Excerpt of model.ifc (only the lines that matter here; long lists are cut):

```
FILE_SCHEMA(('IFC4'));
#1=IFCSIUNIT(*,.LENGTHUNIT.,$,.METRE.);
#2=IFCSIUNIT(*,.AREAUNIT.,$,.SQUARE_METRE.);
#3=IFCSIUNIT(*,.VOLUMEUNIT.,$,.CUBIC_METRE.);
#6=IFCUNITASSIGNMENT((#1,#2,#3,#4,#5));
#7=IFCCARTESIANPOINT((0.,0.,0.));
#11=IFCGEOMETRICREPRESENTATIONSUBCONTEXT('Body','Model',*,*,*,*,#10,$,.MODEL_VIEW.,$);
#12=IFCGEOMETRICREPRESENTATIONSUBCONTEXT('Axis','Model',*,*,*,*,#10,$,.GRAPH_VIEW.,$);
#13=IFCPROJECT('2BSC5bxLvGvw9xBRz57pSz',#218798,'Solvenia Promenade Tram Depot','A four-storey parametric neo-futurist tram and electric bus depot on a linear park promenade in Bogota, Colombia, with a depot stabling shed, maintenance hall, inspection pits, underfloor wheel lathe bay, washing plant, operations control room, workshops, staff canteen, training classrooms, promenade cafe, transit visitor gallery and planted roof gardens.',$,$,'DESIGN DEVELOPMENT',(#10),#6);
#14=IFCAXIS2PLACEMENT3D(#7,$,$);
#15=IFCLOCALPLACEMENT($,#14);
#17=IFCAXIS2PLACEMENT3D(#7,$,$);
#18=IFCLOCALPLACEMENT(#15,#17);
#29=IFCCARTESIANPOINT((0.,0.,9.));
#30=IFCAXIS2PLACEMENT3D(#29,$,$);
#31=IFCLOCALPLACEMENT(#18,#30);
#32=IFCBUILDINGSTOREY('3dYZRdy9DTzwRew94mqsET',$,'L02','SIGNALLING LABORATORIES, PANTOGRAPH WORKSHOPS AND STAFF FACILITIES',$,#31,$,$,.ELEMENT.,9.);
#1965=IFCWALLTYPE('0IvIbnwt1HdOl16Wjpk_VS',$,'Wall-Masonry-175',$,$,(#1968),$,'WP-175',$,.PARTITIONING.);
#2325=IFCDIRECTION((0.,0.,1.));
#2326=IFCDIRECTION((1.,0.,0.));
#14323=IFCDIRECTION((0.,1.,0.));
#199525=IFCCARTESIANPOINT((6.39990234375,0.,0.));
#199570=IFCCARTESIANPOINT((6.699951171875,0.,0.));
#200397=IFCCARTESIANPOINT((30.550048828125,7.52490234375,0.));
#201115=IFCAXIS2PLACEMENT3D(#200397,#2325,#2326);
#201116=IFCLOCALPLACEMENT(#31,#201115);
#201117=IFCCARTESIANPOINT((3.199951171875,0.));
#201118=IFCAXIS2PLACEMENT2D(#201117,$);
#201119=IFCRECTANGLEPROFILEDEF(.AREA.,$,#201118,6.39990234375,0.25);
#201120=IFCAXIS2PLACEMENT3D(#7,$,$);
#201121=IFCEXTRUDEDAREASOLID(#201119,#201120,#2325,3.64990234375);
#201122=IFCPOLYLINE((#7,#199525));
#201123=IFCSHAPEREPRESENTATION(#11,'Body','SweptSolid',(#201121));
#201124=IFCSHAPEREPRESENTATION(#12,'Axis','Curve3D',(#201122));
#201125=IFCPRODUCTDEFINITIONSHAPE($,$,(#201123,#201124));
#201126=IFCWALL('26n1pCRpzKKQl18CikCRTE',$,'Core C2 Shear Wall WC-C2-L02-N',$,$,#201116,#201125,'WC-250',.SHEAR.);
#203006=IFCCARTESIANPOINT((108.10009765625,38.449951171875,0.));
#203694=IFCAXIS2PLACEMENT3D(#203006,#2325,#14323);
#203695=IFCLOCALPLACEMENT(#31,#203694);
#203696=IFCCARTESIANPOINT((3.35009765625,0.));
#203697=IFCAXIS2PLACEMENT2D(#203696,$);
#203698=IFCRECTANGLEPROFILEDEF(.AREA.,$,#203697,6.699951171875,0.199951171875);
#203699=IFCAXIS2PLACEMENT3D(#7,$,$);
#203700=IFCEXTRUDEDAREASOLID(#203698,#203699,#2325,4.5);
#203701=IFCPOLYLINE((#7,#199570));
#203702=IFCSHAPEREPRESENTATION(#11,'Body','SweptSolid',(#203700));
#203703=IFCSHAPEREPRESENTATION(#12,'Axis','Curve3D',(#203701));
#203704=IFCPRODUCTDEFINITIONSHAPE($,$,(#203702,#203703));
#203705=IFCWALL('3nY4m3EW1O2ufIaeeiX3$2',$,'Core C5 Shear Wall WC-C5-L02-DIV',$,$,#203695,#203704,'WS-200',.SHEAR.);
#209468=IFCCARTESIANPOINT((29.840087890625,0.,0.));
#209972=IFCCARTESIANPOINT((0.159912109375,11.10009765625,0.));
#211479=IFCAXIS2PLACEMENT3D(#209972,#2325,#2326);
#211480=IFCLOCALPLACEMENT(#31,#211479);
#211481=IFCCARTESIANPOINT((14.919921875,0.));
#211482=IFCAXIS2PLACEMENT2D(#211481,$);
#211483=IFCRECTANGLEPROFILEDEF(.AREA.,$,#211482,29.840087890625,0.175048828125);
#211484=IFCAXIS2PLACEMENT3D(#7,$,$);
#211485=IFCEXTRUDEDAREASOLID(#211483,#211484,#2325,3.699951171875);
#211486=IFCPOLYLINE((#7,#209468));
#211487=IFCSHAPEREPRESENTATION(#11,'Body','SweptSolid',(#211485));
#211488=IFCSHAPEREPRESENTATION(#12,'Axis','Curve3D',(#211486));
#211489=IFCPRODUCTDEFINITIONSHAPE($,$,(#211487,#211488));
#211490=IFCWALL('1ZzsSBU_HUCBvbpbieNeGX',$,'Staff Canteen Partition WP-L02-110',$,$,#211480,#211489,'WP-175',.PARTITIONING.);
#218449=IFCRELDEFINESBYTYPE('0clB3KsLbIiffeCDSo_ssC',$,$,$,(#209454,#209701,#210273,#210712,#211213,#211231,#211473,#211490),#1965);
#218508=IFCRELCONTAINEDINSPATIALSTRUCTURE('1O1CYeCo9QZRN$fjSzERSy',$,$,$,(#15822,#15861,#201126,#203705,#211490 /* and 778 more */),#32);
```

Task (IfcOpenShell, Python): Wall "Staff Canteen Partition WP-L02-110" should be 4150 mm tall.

```python
import ifcopenshell
import ifcopenshell.geom
import ifcopenshell.util.representation
import ifcopenshell.util.shape

model = ifcopenshell.open("model.ifc")
settings = ifcopenshell.geom.settings()


def volume(element):
    """Net volume in cubic metres, openings subtracted."""
    shape = ifcopenshell.geom.create_shape(settings, element)
    return ifcopenshell.util.shape.get_volume(shape.geometry)


wall = model.by_guid("1ZzsSBU_HUCBvbpbieNeGX")
before = volume(wall)

body = ifcopenshell.util.representation.get_representation(wall, "Model", "Body")
solid = body.Items[0]
old_height = solid.Depth
solid.Depth = 4.15
after = volume(wall)

print(f"height {old_height:g} -> {solid.Depth:g}, volume {before:.3f} -> {after:.3f} m3")

model.write("model_v2.ifc")
```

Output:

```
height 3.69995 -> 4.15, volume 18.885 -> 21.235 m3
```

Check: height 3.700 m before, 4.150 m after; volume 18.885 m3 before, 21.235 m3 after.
